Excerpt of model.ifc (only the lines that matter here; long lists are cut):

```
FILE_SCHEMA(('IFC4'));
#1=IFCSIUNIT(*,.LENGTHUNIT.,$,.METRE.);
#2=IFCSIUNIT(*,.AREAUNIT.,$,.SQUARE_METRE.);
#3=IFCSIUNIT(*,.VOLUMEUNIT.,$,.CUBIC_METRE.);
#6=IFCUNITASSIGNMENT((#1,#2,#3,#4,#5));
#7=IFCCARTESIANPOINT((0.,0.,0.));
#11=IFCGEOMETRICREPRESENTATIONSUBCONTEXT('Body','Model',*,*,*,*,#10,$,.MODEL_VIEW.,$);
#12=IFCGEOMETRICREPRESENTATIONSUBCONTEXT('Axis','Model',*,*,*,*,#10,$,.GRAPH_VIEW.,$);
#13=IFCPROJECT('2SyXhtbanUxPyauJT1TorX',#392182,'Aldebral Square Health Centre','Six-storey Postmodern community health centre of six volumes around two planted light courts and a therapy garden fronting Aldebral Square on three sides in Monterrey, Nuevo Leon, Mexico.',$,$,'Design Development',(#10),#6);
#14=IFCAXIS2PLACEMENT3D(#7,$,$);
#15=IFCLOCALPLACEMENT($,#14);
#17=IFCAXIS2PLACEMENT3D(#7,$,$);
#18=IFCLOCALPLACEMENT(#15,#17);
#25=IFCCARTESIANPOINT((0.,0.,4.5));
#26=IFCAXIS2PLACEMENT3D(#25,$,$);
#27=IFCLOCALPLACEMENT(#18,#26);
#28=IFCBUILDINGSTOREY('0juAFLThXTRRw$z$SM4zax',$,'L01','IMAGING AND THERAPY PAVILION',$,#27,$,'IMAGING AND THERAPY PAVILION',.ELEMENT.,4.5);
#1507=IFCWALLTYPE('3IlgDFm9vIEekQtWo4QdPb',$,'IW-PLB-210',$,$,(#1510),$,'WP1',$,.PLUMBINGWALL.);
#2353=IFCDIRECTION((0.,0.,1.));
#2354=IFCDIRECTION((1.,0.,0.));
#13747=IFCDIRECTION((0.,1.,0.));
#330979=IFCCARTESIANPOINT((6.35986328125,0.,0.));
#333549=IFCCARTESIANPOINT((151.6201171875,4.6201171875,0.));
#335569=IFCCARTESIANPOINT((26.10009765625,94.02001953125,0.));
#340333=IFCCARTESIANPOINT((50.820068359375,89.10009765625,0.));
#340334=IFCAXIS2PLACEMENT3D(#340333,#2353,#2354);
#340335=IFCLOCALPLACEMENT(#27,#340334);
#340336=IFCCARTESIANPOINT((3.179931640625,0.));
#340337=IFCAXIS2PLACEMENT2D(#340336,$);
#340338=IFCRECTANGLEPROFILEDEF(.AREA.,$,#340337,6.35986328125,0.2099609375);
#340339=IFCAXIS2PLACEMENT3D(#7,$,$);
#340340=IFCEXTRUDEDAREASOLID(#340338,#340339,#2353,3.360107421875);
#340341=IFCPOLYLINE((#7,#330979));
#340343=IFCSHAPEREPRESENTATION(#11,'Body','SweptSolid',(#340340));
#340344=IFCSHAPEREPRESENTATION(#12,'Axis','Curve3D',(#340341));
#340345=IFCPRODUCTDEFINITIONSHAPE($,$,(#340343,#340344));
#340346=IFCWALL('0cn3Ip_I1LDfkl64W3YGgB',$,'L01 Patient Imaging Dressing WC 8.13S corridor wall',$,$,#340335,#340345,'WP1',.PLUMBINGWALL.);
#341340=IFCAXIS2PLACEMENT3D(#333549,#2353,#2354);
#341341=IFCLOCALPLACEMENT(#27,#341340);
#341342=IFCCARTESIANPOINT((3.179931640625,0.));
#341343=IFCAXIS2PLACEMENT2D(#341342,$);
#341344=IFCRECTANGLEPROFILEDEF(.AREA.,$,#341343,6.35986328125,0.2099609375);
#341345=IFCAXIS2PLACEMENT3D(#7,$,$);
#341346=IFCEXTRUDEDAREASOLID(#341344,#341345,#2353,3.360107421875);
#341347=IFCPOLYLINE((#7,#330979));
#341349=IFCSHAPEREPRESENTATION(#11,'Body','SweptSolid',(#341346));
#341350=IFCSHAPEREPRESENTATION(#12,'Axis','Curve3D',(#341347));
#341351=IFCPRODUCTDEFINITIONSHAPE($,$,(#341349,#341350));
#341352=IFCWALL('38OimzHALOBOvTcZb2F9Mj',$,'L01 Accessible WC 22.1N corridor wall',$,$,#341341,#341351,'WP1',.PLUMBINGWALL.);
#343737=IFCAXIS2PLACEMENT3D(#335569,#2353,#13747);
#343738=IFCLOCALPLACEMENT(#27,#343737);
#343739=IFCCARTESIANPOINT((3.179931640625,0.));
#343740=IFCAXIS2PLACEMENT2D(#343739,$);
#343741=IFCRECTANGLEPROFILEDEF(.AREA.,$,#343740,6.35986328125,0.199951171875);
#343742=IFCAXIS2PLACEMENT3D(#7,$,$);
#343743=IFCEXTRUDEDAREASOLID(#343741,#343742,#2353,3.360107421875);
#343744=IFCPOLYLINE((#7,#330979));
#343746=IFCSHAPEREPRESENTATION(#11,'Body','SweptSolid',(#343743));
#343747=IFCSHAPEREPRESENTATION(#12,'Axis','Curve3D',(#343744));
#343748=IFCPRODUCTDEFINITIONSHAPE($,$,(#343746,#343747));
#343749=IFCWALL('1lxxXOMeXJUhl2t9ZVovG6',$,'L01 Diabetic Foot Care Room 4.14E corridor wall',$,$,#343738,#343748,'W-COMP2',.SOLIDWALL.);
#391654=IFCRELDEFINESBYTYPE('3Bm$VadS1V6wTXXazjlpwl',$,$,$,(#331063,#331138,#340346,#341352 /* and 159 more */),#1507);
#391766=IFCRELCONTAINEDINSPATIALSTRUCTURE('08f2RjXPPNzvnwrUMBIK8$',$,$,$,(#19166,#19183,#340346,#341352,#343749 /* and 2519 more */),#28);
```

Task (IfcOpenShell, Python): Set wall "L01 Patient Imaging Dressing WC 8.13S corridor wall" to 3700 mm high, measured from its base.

```python
import ifcopenshell
import ifcopenshell.geom
import ifcopenshell.util.representation
import ifcopenshell.util.shape

model = ifcopenshell.open("model.ifc")
settings = ifcopenshell.geom.settings()


def volume(element):
    """Net volume in cubic metres, openings subtracted."""
    shape = ifcopenshell.geom.create_shape(settings, element)
    return ifcopenshell.util.shape.get_volume(shape.geometry)


wall = model.by_guid("0cn3Ip_I1LDfkl64W3YGgB")
before = volume(wall)

body = ifcopenshell.util.representation.get_representation(wall, "Model", "Body")
solid = body.Items[0]
old_height = solid.Depth
solid.Depth = 3.7
after = volume(wall)

print(f"height {old_height:g} -> {solid.Depth:g}, volume {before:.3f} -> {after:.3f} m3")

model.write("model-out.ifc")
```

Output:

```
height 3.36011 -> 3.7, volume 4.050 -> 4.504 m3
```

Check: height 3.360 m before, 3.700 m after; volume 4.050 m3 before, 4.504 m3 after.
